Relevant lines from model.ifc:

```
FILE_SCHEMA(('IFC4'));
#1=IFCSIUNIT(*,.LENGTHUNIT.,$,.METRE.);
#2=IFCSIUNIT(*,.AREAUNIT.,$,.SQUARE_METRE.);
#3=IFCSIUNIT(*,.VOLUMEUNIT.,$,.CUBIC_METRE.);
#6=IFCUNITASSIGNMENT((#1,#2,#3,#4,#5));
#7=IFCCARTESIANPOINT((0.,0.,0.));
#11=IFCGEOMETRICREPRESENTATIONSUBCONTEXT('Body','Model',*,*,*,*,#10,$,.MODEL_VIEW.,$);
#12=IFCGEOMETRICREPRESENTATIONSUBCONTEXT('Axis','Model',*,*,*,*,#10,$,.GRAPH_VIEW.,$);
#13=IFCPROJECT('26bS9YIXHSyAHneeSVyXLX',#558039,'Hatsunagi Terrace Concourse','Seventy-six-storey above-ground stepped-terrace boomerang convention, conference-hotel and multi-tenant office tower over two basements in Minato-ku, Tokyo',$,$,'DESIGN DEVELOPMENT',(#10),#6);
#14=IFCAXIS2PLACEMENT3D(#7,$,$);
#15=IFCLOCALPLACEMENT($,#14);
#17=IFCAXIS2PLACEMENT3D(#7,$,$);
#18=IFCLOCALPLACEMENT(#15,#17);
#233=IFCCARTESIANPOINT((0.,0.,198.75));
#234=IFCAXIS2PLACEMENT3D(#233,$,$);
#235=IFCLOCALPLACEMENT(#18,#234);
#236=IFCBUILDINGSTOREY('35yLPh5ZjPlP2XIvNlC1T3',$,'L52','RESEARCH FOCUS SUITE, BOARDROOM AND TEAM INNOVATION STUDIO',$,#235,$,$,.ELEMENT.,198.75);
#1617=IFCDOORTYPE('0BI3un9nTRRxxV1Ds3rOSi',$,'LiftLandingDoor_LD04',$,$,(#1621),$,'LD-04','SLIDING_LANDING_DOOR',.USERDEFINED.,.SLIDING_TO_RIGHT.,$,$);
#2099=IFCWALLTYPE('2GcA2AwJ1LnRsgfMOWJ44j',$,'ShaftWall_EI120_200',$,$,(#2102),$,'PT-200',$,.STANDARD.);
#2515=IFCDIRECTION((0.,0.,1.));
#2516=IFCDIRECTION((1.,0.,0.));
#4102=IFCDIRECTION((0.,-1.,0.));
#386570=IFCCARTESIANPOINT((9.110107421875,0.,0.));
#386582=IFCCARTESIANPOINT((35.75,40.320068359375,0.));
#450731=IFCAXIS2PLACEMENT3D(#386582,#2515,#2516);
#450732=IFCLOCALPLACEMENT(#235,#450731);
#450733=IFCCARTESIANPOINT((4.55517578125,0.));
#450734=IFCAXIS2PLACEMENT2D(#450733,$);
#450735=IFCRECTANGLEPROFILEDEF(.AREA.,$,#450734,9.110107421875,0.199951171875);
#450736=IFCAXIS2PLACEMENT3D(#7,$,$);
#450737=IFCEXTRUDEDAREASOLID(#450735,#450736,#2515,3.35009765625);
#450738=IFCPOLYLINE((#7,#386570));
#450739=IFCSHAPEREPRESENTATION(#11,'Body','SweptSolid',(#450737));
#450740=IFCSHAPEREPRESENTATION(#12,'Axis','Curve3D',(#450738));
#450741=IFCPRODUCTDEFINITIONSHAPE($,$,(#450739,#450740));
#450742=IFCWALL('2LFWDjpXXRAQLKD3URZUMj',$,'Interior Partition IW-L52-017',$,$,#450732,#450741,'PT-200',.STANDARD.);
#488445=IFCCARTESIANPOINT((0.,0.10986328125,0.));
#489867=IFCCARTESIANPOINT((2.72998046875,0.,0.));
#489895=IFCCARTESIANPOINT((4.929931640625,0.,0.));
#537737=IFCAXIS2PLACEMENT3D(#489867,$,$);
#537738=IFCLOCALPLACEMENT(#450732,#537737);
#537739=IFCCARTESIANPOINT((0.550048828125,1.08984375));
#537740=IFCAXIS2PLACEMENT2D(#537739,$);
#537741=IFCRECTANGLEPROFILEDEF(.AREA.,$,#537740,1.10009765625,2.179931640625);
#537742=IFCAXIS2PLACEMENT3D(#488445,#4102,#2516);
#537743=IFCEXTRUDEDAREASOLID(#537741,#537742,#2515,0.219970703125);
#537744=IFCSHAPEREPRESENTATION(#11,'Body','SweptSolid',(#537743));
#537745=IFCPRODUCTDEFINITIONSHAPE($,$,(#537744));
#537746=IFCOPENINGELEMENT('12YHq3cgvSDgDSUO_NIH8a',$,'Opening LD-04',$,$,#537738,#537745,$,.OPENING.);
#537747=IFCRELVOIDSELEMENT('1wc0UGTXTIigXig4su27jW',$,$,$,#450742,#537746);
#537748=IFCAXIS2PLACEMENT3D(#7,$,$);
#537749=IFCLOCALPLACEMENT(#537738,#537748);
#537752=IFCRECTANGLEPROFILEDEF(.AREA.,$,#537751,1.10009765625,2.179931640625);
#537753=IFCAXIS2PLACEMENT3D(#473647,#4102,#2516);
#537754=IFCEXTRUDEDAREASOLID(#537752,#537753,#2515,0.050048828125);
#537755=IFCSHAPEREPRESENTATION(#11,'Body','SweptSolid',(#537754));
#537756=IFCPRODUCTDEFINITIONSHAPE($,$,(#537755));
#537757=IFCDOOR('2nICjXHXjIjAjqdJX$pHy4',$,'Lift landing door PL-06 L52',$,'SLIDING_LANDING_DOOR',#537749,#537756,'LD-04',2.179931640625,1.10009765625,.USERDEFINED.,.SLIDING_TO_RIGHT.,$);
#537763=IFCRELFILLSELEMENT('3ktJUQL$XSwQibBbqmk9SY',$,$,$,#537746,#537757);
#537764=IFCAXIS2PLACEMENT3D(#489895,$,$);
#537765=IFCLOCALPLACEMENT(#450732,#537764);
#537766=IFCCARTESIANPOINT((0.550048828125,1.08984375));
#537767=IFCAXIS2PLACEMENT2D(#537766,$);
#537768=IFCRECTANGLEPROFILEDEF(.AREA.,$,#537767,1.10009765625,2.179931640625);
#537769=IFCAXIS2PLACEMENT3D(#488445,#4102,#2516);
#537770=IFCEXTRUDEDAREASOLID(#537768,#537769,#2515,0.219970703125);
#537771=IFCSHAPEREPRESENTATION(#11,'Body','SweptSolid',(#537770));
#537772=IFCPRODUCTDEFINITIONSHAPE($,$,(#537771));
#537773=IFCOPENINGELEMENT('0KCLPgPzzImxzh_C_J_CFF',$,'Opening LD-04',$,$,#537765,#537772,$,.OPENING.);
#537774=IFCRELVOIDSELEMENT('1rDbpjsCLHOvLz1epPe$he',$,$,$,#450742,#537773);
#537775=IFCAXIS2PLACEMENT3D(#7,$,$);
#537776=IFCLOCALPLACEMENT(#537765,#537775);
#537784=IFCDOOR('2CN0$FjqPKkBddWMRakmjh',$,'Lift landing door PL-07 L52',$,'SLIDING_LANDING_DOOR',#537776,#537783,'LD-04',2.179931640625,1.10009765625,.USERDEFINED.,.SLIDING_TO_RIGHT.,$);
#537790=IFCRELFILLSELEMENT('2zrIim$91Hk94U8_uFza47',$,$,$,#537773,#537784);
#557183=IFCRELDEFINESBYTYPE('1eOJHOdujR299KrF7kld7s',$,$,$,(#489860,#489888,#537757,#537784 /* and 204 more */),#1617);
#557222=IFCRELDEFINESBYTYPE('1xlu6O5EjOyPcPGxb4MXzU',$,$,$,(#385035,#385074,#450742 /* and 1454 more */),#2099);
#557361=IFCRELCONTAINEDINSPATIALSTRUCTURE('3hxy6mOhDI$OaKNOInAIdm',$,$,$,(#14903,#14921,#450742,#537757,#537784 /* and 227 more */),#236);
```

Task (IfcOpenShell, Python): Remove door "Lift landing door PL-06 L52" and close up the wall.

```python
import ifcopenshell
import ifcopenshell.api.feature
import ifcopenshell.api.root
import ifcopenshell.geom
import ifcopenshell.util.shape

model = ifcopenshell.open("model.ifc")
settings = ifcopenshell.geom.settings()


def volume(element):
    """Net volume in cubic metres, openings subtracted."""
    shape = ifcopenshell.geom.create_shape(settings, element)
    return ifcopenshell.util.shape.get_volume(shape.geometry)


door = model.by_guid("2nICjXHXjIjAjqdJX$pHy4")
opening = door.FillsVoids[0].RelatingOpeningElement
wall = opening.VoidsElements[0].RelatingBuildingElement
before = volume(wall)

ifcopenshell.api.root.remove_product(model, product=door)
ifcopenshell.api.feature.remove_feature(model, feature=opening)

after = volume(wall)

print(f"wall volume {before:.3f} -> {after:.3f} m3")

model.write("model_updated.ifc")
```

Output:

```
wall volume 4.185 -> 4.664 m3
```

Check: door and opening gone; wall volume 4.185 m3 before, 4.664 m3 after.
